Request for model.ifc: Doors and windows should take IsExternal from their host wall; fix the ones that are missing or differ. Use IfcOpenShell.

First a look at what the model holds.

```python
import ifcopenshell
import ifcopenshell.util.element

model = ifcopenshell.open("model.ifc")
print(model.schema)
seen = {}
for e in model.by_type("IfcDoor") + model.by_type("IfcWindow"):
    if not e.FillsVoids:
        continue
    host = e.FillsVoids[0].RelatingOpeningElement.VoidsElements[0].RelatingBuildingElement
    own = ifcopenshell.util.element.get_pset(e, f"Pset_{e.is_a()[3:].removesuffix('StandardCase')}Common", "IsExternal")
    wall = ifcopenshell.util.element.get_pset(host, "Pset_WallCommon", "IsExternal")
    seen[e.is_a(), own, wall] = seen.get((e.is_a(), own, wall), 0) + 1
for (cls, own, wall), count in sorted(seen.items(), key=str):
    print(count, cls, "IsExternal:", own, "| host wall:", wall)
```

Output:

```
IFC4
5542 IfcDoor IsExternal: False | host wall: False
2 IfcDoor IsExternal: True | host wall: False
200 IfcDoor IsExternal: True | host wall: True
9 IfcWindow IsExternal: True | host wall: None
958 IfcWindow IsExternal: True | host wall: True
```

```python
import ifcopenshell
import ifcopenshell.api.pset
import ifcopenshell.util.element

model = ifcopenshell.open("model.ifc")

count = 0
for ifc_class, pset_name in (("IfcDoor", "Pset_DoorCommon"), ("IfcWindow", "Pset_WindowCommon")):
    for e in model.by_type(ifc_class):
        if not e.FillsVoids:
            continue
        host = e.FillsVoids[0].RelatingOpeningElement.VoidsElements[0].RelatingBuildingElement
        external = ifcopenshell.util.element.get_pset(host, "Pset_WallCommon", "IsExternal")
        if external is None or ifcopenshell.util.element.get_pset(e, pset_name, "IsExternal") == external:
            continue
        pset = ifcopenshell.api.pset.add_pset(model, product=e, name=pset_name)
        ifcopenshell.api.pset.edit_pset(model, pset=pset, properties={"IsExternal": external})
        count += 1

print(count, "updated")

model.write("model_edited.ifc")
```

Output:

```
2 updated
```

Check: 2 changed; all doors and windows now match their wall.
